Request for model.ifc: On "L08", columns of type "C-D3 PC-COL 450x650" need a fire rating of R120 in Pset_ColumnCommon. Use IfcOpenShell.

First a look at what the model holds.

```python
import ifcopenshell
import ifcopenshell.util.element

model = ifcopenshell.open("model.ifc")
print(model.schema)
storey = next(s for s in model.by_type("IfcBuildingStorey") if s.Name == "L08")
columns = [e for e in ifcopenshell.util.element.get_decomposition(storey) if e.is_a("IfcColumn")]
seen = {}
for e in columns:
    element_type = ifcopenshell.util.element.get_type(e)
    key = (element_type.Name if element_type != e and element_type else None, ifcopenshell.util.element.get_pset(e, "Pset_ColumnCommon", "FireRating"))
    seen[key] = seen.get(key, 0) + 1
for (name, value), count in sorted(seen.items(), key=str):
    print(count, "x", name, "|", value)
```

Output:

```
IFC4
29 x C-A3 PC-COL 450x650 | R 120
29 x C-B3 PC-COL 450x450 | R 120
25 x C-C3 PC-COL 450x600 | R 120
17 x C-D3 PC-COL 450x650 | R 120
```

```python
import ifcopenshell
import ifcopenshell.api.pset
import ifcopenshell.util.element

model = ifcopenshell.open("model.ifc")

storey = next(s for s in model.by_type("IfcBuildingStorey") if s.Name == "L08")
columns = [e for e in ifcopenshell.util.element.get_decomposition(storey) if e.is_a("IfcColumn")]

count = 0
for e in columns:
    element_type = ifcopenshell.util.element.get_type(e)
    if element_type in (None, e) or element_type.Name != "C-D3 PC-COL 450x650":
        continue
    # add_pset returns the element's existing set when there is one.
    pset = ifcopenshell.api.pset.add_pset(model, product=e, name="Pset_ColumnCommon")
    ifcopenshell.api.pset.edit_pset(model, pset=pset, properties={"FireRating": "R120"})
    count += 1

print(count, "columns updated")

model.write("model-out.ifc")
```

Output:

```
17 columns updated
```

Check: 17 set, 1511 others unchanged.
